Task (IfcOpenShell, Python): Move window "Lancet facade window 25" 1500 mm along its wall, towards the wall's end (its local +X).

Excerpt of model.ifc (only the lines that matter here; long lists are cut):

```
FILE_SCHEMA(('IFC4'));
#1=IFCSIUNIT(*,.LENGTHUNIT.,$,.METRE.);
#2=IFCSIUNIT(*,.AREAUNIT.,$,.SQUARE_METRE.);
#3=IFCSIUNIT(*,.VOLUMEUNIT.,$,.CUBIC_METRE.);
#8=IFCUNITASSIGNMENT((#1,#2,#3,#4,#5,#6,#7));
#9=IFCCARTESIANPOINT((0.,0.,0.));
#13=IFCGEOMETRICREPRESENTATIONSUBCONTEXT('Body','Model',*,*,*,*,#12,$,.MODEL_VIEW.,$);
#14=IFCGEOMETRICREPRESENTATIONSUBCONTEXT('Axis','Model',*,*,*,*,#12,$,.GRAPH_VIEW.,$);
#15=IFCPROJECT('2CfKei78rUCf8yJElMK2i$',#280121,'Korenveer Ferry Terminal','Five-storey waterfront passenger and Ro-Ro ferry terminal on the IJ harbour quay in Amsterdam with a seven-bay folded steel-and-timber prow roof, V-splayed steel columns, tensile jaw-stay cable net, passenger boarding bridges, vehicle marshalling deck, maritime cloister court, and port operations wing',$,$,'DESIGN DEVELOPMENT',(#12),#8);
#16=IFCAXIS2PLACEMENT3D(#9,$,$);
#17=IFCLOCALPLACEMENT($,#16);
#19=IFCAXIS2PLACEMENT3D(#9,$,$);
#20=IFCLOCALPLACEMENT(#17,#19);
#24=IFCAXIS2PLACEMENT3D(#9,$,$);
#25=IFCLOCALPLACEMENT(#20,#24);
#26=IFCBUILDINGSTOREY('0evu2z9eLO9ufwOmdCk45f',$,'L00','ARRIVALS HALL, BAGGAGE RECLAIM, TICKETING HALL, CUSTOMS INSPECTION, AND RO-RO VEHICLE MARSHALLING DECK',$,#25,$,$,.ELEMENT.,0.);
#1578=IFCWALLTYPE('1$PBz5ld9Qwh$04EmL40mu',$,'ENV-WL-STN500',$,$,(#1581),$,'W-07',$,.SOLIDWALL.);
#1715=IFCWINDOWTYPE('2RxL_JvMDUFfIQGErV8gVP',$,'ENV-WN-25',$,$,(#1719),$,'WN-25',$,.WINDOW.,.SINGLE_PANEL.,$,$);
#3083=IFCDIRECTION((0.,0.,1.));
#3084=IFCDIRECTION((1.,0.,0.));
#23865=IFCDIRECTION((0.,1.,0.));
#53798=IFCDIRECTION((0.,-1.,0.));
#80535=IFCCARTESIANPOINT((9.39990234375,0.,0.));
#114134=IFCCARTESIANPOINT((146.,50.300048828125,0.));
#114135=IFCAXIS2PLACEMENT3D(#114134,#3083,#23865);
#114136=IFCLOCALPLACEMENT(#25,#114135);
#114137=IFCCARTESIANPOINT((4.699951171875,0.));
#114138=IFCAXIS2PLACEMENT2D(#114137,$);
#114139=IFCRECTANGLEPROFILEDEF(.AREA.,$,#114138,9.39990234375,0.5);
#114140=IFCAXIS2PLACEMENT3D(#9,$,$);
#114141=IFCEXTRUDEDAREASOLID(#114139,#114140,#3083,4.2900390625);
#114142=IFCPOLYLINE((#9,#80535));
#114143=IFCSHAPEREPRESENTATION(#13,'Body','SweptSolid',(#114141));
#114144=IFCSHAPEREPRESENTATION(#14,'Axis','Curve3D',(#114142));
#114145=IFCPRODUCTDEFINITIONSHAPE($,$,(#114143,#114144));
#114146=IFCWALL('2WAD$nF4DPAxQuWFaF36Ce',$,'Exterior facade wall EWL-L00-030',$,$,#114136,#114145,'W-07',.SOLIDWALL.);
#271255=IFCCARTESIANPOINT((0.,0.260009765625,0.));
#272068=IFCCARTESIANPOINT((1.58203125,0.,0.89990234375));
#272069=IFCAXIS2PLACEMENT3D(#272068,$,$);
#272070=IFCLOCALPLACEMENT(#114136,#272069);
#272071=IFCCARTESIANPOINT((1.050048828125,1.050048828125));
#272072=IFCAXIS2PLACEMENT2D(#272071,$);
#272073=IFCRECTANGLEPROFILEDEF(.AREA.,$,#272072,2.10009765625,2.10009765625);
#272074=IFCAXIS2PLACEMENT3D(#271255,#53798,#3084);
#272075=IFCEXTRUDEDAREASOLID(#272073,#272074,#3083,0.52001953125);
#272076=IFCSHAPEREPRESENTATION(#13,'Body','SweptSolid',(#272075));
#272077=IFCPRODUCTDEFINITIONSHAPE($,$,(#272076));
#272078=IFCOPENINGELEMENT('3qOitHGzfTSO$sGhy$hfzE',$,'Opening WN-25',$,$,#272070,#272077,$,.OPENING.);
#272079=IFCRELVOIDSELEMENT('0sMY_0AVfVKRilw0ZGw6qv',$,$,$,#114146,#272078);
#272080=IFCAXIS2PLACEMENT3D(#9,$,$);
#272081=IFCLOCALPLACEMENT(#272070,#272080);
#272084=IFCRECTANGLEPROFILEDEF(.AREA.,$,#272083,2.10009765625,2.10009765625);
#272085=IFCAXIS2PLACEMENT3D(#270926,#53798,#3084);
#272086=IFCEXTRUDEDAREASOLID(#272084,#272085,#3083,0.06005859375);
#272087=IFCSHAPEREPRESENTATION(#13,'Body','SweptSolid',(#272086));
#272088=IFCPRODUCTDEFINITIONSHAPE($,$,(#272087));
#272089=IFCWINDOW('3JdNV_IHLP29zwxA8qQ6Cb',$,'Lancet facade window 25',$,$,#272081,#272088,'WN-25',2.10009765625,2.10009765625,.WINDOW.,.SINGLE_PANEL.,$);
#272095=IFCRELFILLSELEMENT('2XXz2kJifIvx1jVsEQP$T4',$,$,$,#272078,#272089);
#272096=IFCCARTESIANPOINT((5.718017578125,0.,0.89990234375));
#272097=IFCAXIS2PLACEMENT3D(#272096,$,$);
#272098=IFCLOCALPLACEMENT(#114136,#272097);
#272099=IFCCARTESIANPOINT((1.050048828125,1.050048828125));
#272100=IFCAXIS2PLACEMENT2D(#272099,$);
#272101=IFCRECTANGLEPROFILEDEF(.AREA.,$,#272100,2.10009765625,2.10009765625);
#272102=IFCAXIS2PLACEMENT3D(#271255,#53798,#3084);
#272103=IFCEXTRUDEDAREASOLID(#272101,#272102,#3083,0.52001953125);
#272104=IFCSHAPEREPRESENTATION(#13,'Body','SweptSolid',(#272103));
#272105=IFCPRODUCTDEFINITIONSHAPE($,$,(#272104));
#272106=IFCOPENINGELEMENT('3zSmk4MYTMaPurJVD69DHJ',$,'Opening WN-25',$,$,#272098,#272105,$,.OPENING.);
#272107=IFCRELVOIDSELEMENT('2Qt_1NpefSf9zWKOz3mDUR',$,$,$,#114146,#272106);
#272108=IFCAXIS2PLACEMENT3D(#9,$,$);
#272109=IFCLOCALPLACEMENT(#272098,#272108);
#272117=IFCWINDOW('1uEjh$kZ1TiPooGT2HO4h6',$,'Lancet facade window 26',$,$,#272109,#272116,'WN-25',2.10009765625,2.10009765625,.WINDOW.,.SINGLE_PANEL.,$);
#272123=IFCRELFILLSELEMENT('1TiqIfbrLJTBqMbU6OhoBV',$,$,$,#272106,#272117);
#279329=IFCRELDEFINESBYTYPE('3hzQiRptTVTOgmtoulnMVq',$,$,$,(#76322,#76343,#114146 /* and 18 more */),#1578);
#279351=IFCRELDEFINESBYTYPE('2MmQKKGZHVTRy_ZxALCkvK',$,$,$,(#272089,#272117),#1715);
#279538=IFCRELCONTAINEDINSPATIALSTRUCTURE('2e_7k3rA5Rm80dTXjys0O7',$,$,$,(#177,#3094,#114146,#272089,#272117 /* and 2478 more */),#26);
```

```python
import ifcopenshell
import ifcopenshell.api.geometry
import ifcopenshell.util.placement
import ifcopenshell.util.unit

model = ifcopenshell.open("model.ifc")
unit_scale = ifcopenshell.util.unit.calculate_unit_scale(model)

window = model.by_guid("3JdNV_IHLP29zwxA8qQ6Cb")
opening = window.FillsVoids[0].RelatingOpeningElement
wall = opening.VoidsElements[0].RelatingBuildingElement

wall_matrix = ifcopenshell.util.placement.get_local_placement(wall.ObjectPlacement)
shift = wall_matrix[:3, 0] * 1.5 / unit_scale
before = ifcopenshell.util.placement.get_local_placement(window.ObjectPlacement)[:3, 3].copy()

# The window is placed relative to its opening, so it follows when the opening moves.
matrix = ifcopenshell.util.placement.get_local_placement(opening.ObjectPlacement)
matrix[:3, 3] += shift
ifcopenshell.api.geometry.edit_object_placement(
    model, product=opening, matrix=matrix, is_si=False, should_transform_children=True
)

after = ifcopenshell.util.placement.get_local_placement(window.ObjectPlacement)[:3, 3]
print("window moved by", (after - before).round(3) + 0.0)

model.write("model_v2.ifc")
```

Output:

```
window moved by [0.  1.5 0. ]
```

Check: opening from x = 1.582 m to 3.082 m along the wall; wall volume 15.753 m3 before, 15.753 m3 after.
